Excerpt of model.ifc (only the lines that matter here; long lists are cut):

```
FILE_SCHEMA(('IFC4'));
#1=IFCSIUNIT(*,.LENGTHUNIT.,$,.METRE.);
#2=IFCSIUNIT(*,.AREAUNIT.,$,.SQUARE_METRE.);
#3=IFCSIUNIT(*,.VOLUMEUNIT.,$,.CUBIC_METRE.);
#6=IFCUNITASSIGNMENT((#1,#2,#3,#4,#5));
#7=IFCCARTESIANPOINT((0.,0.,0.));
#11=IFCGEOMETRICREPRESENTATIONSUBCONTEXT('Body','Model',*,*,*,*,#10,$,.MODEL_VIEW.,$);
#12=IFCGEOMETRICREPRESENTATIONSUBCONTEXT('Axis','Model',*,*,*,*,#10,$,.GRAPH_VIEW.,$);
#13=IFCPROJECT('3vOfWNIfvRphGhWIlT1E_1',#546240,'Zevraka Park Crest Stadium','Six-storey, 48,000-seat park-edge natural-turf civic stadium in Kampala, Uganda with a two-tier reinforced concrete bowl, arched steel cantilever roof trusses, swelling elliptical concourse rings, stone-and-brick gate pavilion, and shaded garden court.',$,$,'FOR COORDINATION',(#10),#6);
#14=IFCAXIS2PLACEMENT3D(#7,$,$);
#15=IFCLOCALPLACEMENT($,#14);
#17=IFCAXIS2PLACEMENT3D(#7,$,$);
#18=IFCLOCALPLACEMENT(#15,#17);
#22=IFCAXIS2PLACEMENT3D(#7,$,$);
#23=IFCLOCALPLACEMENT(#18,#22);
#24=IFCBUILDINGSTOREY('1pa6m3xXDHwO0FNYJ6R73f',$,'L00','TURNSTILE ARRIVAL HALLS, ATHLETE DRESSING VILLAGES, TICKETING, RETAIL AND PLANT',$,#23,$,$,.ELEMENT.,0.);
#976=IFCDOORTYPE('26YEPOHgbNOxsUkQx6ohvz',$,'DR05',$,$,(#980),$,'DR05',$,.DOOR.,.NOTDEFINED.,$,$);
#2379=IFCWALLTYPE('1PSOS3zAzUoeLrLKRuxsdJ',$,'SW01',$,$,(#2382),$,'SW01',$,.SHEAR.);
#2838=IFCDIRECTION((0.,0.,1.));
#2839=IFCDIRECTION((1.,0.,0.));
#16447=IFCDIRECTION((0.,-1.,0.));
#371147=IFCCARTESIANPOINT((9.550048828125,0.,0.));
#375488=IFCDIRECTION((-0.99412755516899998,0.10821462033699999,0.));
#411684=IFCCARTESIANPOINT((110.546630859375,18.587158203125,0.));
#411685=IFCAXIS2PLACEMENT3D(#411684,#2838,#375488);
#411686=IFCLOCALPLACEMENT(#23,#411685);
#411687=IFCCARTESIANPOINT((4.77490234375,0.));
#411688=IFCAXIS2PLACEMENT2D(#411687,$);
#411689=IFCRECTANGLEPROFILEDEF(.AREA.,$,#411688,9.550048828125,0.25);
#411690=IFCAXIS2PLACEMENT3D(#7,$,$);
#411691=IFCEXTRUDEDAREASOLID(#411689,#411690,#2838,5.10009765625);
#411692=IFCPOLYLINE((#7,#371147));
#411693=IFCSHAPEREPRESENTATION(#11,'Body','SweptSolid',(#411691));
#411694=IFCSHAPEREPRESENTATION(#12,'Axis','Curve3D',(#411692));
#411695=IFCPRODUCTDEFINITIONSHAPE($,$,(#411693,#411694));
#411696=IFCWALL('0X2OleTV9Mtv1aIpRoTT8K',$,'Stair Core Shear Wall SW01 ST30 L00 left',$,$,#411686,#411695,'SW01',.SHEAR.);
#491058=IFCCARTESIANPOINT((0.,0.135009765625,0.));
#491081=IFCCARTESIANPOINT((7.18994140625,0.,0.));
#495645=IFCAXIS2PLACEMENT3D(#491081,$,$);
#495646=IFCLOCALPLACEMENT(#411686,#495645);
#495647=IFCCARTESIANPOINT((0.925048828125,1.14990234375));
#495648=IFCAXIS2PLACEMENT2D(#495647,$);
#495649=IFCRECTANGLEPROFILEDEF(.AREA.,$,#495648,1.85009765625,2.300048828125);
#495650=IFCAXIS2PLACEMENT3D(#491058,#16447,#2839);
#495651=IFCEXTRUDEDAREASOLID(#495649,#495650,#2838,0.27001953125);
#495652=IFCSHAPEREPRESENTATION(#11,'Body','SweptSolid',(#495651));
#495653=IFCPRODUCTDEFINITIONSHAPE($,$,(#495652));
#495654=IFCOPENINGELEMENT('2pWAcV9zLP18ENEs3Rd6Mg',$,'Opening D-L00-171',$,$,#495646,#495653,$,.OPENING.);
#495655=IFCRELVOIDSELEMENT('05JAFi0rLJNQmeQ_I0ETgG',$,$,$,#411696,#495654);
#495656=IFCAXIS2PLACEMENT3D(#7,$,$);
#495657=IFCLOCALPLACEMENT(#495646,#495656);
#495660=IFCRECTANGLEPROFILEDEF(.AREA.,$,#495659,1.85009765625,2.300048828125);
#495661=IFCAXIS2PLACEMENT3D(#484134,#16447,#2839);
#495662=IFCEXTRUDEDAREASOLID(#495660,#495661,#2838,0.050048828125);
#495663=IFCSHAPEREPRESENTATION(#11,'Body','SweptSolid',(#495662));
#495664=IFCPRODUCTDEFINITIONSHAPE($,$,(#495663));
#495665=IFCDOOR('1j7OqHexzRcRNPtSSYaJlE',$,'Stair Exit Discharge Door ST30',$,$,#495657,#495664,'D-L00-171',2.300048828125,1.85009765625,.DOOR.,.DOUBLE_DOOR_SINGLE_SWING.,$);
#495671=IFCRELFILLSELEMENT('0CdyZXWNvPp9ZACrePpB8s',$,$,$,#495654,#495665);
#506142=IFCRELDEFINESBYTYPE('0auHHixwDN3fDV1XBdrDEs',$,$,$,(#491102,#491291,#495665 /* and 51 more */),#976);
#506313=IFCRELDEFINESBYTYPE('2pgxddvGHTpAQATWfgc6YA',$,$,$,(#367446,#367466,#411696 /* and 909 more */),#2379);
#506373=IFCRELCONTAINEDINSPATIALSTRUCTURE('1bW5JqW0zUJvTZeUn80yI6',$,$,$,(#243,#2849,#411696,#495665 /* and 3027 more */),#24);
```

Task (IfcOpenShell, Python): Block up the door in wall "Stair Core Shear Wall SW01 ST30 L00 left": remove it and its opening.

```python
import ifcopenshell
import ifcopenshell.api.feature
import ifcopenshell.api.root
import ifcopenshell.geom
import ifcopenshell.util.shape

model = ifcopenshell.open("model.ifc")
settings = ifcopenshell.geom.settings()


def volume(element):
    """Net volume in cubic metres, openings subtracted."""
    shape = ifcopenshell.geom.create_shape(settings, element)
    return ifcopenshell.util.shape.get_volume(shape.geometry)


door = model.by_guid("1j7OqHexzRcRNPtSSYaJlE")
opening = door.FillsVoids[0].RelatingOpeningElement
wall = opening.VoidsElements[0].RelatingBuildingElement
before = volume(wall)

ifcopenshell.api.root.remove_product(model, product=door)
ifcopenshell.api.feature.remove_feature(model, feature=opening)

after = volume(wall)

print(f"wall volume {before:.3f} -> {after:.3f} m3")

model.write("model_v2.ifc")
```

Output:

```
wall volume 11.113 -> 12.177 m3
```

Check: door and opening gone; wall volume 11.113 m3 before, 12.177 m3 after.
